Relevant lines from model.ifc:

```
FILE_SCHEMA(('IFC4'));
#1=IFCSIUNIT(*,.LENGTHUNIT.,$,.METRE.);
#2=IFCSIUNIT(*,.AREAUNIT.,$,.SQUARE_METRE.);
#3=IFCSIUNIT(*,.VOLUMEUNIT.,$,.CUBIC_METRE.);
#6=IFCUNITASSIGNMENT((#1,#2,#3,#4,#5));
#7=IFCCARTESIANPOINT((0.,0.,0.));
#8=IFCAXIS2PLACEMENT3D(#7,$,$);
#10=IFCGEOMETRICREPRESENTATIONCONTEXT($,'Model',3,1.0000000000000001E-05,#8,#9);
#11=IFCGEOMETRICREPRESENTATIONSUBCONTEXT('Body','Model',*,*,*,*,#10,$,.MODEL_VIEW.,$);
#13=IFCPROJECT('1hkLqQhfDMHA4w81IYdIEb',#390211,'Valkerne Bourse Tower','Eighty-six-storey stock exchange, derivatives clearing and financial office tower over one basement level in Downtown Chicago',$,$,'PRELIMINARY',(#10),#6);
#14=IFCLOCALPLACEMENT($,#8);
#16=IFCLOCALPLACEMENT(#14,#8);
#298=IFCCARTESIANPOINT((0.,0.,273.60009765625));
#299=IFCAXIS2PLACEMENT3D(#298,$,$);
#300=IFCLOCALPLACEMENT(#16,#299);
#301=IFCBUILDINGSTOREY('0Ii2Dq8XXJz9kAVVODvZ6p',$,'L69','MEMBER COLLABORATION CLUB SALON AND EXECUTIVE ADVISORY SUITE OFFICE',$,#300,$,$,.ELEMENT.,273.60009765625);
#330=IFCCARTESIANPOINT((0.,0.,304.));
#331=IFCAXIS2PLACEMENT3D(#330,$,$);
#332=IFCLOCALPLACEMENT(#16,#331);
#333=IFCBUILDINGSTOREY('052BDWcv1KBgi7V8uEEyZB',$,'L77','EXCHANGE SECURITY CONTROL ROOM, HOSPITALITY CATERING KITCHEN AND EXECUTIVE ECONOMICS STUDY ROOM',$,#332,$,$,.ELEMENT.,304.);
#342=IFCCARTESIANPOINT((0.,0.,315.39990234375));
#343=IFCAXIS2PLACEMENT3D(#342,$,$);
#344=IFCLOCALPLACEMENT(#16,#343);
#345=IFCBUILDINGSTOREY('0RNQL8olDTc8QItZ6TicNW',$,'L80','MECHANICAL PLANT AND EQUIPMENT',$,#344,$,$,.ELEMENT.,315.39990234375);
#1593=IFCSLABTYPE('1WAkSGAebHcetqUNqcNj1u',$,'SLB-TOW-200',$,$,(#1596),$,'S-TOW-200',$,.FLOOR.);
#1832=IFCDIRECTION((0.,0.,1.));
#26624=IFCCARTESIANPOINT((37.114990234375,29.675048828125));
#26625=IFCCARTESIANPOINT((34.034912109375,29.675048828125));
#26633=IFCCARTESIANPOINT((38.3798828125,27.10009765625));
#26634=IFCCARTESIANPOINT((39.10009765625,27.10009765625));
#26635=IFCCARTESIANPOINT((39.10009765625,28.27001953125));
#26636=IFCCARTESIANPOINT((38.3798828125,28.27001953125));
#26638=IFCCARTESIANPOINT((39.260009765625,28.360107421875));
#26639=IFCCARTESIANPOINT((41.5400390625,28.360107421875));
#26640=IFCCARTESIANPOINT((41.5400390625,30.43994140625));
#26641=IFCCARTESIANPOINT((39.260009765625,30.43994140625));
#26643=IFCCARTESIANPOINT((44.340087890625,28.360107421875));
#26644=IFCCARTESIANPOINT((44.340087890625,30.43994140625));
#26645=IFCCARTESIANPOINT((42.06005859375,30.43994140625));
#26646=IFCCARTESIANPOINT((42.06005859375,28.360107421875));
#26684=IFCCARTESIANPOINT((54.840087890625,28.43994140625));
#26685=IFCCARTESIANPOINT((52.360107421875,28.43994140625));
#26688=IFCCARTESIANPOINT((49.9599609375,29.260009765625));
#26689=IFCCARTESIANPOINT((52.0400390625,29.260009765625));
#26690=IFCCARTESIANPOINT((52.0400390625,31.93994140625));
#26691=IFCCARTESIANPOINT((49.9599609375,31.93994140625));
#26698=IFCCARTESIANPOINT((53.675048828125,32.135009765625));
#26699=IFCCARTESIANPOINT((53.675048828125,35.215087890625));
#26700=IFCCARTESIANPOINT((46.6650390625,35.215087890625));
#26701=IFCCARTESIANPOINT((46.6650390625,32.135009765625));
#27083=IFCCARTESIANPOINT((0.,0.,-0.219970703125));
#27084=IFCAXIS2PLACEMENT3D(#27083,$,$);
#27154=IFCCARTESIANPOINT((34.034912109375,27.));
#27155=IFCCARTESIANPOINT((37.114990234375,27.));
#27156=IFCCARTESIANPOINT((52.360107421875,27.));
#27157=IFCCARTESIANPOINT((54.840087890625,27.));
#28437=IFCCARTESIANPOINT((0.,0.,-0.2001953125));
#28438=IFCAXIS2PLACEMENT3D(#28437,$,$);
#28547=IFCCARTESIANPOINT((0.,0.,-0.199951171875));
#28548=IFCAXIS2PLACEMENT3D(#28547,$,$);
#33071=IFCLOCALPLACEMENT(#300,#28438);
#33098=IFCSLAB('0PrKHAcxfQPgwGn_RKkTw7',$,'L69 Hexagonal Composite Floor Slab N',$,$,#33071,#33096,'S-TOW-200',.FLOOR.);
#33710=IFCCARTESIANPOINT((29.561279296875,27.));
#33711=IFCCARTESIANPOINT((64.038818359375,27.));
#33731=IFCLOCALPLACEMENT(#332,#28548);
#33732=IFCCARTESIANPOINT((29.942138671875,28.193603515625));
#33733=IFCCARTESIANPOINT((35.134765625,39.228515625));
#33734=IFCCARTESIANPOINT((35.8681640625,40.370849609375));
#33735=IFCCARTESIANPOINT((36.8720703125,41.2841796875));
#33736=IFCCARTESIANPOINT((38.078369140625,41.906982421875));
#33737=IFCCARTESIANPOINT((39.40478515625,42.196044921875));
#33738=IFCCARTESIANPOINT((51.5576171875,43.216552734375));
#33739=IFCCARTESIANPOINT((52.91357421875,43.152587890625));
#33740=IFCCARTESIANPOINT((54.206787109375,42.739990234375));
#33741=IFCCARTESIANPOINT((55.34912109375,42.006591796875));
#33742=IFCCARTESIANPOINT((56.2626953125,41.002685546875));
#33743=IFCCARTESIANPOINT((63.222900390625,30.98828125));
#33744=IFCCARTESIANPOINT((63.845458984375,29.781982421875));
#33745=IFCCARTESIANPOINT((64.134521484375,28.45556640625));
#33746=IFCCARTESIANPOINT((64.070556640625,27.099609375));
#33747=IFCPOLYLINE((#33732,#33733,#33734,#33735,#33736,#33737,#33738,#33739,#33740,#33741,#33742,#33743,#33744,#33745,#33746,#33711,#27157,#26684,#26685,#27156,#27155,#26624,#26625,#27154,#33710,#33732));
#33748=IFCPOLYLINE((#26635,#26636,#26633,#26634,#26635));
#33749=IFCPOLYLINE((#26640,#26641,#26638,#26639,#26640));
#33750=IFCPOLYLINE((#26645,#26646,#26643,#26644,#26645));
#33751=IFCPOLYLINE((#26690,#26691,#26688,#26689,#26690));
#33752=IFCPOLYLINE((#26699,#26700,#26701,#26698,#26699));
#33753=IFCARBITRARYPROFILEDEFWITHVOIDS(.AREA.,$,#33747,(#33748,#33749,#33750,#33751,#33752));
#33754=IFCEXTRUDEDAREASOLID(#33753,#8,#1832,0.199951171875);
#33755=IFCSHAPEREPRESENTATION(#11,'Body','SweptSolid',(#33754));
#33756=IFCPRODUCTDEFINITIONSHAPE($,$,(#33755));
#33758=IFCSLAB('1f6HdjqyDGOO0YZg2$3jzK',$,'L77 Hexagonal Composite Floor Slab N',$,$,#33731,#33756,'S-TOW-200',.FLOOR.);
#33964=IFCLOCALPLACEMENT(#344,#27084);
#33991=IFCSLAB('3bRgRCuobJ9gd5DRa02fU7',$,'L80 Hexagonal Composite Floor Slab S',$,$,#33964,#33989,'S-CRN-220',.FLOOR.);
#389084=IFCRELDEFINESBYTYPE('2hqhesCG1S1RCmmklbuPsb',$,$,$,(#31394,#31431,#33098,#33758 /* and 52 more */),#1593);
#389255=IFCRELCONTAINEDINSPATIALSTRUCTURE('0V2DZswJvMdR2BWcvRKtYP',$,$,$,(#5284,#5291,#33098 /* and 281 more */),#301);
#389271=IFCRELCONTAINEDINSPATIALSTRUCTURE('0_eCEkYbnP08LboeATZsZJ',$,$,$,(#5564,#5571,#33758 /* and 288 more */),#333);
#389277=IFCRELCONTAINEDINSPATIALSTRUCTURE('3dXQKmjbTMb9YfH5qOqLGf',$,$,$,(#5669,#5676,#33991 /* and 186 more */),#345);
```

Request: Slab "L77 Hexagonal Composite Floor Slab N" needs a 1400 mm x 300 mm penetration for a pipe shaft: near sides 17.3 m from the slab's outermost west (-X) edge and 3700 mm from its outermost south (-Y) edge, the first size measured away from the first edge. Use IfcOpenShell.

```python
import numpy as np
import ifcopenshell
import ifcopenshell.api.feature
import ifcopenshell.api.geometry
import ifcopenshell.api.root
import ifcopenshell.geom
import ifcopenshell.util.placement
import ifcopenshell.util.representation
import ifcopenshell.util.shape
import ifcopenshell.util.unit

model = ifcopenshell.open("model.ifc")
unit_scale = ifcopenshell.util.unit.calculate_unit_scale(model)
settings = ifcopenshell.geom.settings()


def volume(element):
    """Net volume in cubic metres, openings subtracted."""
    shape = ifcopenshell.geom.create_shape(settings, element)
    return ifcopenshell.util.shape.get_volume(shape.geometry)


slab = model.by_guid("1f6HdjqyDGOO0YZg2$3jzK")
before = volume(slab)

# Extent in the slab's own axes, in metres. The edges named are its -X and -Y sides.
slab_shape = ifcopenshell.geom.create_shape(settings, slab)
vertices = ifcopenshell.util.shape.get_vertices(slab_shape.geometry)
x_min, y_min, bottom = vertices.min(axis=0)
top = vertices[:, 2].max()

opening = ifcopenshell.api.root.create_entity(model, ifc_class="IfcOpeningElement", name="Pipe shaft opening", predefined_type="OPENING")
context = ifcopenshell.util.representation.get_context(model, "Model", "Body", "MODEL_VIEW")
width, depth = 1.4, 0.3
outline = [(0.0, 0.0), (width, 0.0), (width, depth), (0.0, depth), (0.0, 0.0)]
# Overshoot both faces by 50 mm so the cut is clean.
shape = ifcopenshell.api.geometry.add_slab_representation(
    model, context=context, depth=top - bottom + 0.1, polyline=outline
)
ifcopenshell.api.geometry.assign_representation(model, product=opening, representation=shape)

matrix = ifcopenshell.util.placement.get_local_placement(slab.ObjectPlacement)
matrix[:, 3] = matrix @ np.append(np.array([x_min + 17.3, y_min + 3.7, bottom - 0.05]) / unit_scale, 1.0)
ifcopenshell.api.geometry.edit_object_placement(model, product=opening, matrix=matrix, is_si=False)
ifcopenshell.api.feature.add_feature(model, feature=opening, element=slab)

after = volume(slab)

print(f"slab volume {before:.3f} -> {after:.3f} m3")

model.write("model_v2.ifc")
```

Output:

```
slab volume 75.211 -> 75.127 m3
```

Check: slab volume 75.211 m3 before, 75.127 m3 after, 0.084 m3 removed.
